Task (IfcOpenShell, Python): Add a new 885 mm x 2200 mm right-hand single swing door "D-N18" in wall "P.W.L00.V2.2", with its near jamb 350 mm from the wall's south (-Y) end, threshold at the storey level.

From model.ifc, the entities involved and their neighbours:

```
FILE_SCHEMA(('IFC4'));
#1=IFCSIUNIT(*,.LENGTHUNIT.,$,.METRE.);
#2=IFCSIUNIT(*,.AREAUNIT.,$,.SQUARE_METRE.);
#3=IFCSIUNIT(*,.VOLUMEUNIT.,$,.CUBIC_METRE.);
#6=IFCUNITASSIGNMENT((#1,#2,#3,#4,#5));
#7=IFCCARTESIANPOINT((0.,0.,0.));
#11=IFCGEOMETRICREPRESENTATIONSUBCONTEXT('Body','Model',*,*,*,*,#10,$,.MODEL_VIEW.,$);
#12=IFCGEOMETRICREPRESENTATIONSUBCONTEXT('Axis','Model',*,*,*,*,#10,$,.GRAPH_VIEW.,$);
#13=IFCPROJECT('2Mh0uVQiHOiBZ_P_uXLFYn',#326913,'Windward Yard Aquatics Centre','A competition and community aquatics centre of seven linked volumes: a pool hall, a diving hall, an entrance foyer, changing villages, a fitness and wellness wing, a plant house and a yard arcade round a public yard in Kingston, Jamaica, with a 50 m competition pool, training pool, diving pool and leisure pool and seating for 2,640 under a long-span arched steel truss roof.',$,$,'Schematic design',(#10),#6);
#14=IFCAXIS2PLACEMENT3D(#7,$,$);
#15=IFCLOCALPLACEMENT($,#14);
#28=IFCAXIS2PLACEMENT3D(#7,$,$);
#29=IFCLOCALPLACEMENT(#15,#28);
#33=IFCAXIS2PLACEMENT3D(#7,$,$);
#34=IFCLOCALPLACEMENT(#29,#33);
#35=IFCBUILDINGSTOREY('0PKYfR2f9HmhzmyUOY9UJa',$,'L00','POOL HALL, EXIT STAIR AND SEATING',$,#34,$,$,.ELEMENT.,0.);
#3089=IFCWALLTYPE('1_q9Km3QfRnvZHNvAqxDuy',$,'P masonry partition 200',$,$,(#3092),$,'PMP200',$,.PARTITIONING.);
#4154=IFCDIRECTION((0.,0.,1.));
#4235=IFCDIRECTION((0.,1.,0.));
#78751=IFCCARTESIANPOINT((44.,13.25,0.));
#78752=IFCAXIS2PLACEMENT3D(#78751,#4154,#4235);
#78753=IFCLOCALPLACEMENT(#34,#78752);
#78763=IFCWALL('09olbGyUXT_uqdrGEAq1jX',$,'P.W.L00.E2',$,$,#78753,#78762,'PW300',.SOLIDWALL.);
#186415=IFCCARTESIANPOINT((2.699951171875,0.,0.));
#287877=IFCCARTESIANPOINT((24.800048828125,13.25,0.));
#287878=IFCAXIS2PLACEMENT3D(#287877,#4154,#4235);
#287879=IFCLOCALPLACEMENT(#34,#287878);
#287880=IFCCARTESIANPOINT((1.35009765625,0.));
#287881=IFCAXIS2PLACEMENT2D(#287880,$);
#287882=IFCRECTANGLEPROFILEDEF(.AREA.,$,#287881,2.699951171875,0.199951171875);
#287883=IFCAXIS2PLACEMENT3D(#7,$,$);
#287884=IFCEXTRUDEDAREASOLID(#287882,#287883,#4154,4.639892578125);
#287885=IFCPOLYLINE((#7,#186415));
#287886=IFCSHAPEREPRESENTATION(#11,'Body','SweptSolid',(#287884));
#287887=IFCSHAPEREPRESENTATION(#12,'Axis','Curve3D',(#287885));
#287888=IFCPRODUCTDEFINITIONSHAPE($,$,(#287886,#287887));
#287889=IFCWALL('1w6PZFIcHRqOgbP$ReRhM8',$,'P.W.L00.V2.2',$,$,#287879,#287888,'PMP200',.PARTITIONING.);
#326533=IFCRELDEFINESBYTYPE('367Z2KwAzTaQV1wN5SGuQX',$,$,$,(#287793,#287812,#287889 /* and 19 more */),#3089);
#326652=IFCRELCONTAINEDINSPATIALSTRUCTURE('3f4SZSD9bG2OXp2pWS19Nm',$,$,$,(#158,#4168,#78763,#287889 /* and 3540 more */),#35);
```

```python
import numpy as np
import ifcopenshell
import ifcopenshell.api.feature
import ifcopenshell.api.geometry
import ifcopenshell.api.root
import ifcopenshell.api.spatial
import ifcopenshell.geom
import ifcopenshell.util.element
import ifcopenshell.util.placement
import ifcopenshell.util.representation
import ifcopenshell.util.shape
import ifcopenshell.util.unit

model = ifcopenshell.open("model.ifc")
unit_scale = ifcopenshell.util.unit.calculate_unit_scale(model)
settings = ifcopenshell.geom.settings()


def volume(element):
    """Net volume in cubic metres, openings subtracted."""
    shape = ifcopenshell.geom.create_shape(settings, element)
    return ifcopenshell.util.shape.get_volume(shape.geometry)


wall = model.by_guid("1w6PZFIcHRqOgbP$ReRhM8")
storey = ifcopenshell.util.element.get_container(wall, ifc_class="IfcBuildingStorey")
context = ifcopenshell.util.representation.get_context(model, "Model", "Body", "MODEL_VIEW")
before = volume(wall)

width, height, from_end, sill = 0.885, 2.2, 0.35, 0.0  # metres

# The wall runs along its own X axis, and the end named is its -X end.
wall_shape = ifcopenshell.geom.create_shape(settings, wall)
x, y, z = ifcopenshell.util.shape.get_vertices(wall_shape.geometry).T
start = x.min() + from_end
face, thickness = float(y.min()), float(y.max() - y.min())
wall_matrix = ifcopenshell.util.placement.get_local_placement(wall.ObjectPlacement)
level = ifcopenshell.util.placement.get_local_placement(storey.ObjectPlacement)[2, 3]


def in_wall(x, y):
    """Placement at x, y metres in the wall's axes, at sill height."""
    matrix = wall_matrix.copy()
    matrix[:, 3] = wall_matrix @ np.array([x / unit_scale, y / unit_scale, 0.0, 1.0])
    matrix[2, 3] = level + sill / unit_scale
    return matrix


# Opening: a box that overshoots both wall faces by 50 mm.
opening = ifcopenshell.api.root.create_entity(model, ifc_class="IfcOpeningElement", predefined_type="OPENING")
box = ifcopenshell.api.geometry.add_wall_representation(
    model, context=context, length=width, height=height, thickness=thickness + 0.1
)
ifcopenshell.api.geometry.assign_representation(model, product=opening, representation=box)
ifcopenshell.api.geometry.edit_object_placement(model, product=opening, matrix=in_wall(start, face - 0.05), is_si=False)
ifcopenshell.api.feature.add_feature(model, feature=opening, element=wall)

door = ifcopenshell.api.root.create_entity(model, ifc_class="IfcDoor", name="D-N18", predefined_type="DOOR")
door.OverallWidth, door.OverallHeight = width / unit_scale, height / unit_scale
door.OperationType = "SINGLE_SWING_RIGHT"
body = ifcopenshell.api.geometry.add_door_representation(
    model,
    context=context,
    overall_width=door.OverallWidth,
    overall_height=door.OverallHeight,
    operation_type="SINGLE_SWING_RIGHT",
    lining_properties={"LiningDepth": thickness / unit_scale, "ThresholdDepth": thickness / unit_scale},
)
ifcopenshell.api.geometry.assign_representation(model, product=door, representation=body)
ifcopenshell.api.spatial.assign_container(model, products=[door], relating_structure=storey)
ifcopenshell.api.feature.add_filling(model, opening=opening, element=door)

# The lining spans the wall, so the door starts at the wall face.
ifcopenshell.api.geometry.edit_object_placement(model, product=door, matrix=in_wall(start, face), is_si=False)

after = volume(wall)

print(f"wall volume {before:.3f} -> {after:.3f} m3")

model.write("model_v2.ifc")
```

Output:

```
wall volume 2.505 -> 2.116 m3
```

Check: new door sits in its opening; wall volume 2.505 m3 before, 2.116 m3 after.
